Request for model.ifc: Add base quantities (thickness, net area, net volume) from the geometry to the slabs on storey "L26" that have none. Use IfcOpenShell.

First a look at what the model holds.

```python
import ifcopenshell
import ifcopenshell.util.element
import ifcopenshell.util.unit

model = ifcopenshell.open("model.ifc")
print(model.schema)
for unit_type in ("LENGTHUNIT", "AREAUNIT", "VOLUMEUNIT"):
    print(unit_type, ifcopenshell.util.unit.calculate_unit_scale(model, unit_type))
storey = next(s for s in model.by_type("IfcBuildingStorey") if s.Name == "L26")
slabs = [e for e in ifcopenshell.util.element.get_decomposition(storey) if e.is_a("IfcSlab")]
for e in sorted(slabs, key=lambda e: e.id()):
    print(e.id(), e.is_a(), e.Name, list(ifcopenshell.util.element.get_psets(e, qtos_only=True)), sep=" | ")
```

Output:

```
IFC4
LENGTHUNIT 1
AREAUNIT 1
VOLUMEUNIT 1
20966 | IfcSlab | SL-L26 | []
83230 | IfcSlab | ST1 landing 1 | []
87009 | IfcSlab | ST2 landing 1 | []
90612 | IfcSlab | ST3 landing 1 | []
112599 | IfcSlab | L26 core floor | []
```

```python
import ifcopenshell
import ifcopenshell.api.pset
import ifcopenshell.geom
import ifcopenshell.util.element
import ifcopenshell.util.shape
import ifcopenshell.util.unit

model = ifcopenshell.open("model.ifc")
unit_scale = ifcopenshell.util.unit.calculate_unit_scale(model)
area_scale = ifcopenshell.util.unit.calculate_unit_scale(model, "AREAUNIT")
volume_scale = ifcopenshell.util.unit.calculate_unit_scale(model, "VOLUMEUNIT")
settings = ifcopenshell.geom.settings()

storey = next(s for s in model.by_type("IfcBuildingStorey") if s.Name == "L26")
slabs = [e for e in ifcopenshell.util.element.get_decomposition(storey) if e.is_a("IfcSlab")]

for e in sorted(slabs, key=lambda e: e.id()):
    if ifcopenshell.util.element.get_psets(e, qtos_only=True, should_inherit=False):
        continue
    # Geometry comes back in metres, in the element's own axes.
    shape = ifcopenshell.geom.create_shape(settings, e)
    values = {
        "Width": ifcopenshell.util.shape.get_z(shape.geometry) / unit_scale,
        "NetArea": ifcopenshell.util.shape.get_footprint_area(shape.geometry) / area_scale,
        "NetVolume": ifcopenshell.util.shape.get_volume(shape.geometry) / volume_scale,
    }
    qto = ifcopenshell.api.pset.add_qto(model, product=e, name="Qto_SlabBaseQuantities")
    ifcopenshell.api.pset.edit_qto(model, qto=qto, properties=values)
    print(e.id(), {k: round(v, 3) for k, v in values.items()})

model.write("model-out.ifc")
```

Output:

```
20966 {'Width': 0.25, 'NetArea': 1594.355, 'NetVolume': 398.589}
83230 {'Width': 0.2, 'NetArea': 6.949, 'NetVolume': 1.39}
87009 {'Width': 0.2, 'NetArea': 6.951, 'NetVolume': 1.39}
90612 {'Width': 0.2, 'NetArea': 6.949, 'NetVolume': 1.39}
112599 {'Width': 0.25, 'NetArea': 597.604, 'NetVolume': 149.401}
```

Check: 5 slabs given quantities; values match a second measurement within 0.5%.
